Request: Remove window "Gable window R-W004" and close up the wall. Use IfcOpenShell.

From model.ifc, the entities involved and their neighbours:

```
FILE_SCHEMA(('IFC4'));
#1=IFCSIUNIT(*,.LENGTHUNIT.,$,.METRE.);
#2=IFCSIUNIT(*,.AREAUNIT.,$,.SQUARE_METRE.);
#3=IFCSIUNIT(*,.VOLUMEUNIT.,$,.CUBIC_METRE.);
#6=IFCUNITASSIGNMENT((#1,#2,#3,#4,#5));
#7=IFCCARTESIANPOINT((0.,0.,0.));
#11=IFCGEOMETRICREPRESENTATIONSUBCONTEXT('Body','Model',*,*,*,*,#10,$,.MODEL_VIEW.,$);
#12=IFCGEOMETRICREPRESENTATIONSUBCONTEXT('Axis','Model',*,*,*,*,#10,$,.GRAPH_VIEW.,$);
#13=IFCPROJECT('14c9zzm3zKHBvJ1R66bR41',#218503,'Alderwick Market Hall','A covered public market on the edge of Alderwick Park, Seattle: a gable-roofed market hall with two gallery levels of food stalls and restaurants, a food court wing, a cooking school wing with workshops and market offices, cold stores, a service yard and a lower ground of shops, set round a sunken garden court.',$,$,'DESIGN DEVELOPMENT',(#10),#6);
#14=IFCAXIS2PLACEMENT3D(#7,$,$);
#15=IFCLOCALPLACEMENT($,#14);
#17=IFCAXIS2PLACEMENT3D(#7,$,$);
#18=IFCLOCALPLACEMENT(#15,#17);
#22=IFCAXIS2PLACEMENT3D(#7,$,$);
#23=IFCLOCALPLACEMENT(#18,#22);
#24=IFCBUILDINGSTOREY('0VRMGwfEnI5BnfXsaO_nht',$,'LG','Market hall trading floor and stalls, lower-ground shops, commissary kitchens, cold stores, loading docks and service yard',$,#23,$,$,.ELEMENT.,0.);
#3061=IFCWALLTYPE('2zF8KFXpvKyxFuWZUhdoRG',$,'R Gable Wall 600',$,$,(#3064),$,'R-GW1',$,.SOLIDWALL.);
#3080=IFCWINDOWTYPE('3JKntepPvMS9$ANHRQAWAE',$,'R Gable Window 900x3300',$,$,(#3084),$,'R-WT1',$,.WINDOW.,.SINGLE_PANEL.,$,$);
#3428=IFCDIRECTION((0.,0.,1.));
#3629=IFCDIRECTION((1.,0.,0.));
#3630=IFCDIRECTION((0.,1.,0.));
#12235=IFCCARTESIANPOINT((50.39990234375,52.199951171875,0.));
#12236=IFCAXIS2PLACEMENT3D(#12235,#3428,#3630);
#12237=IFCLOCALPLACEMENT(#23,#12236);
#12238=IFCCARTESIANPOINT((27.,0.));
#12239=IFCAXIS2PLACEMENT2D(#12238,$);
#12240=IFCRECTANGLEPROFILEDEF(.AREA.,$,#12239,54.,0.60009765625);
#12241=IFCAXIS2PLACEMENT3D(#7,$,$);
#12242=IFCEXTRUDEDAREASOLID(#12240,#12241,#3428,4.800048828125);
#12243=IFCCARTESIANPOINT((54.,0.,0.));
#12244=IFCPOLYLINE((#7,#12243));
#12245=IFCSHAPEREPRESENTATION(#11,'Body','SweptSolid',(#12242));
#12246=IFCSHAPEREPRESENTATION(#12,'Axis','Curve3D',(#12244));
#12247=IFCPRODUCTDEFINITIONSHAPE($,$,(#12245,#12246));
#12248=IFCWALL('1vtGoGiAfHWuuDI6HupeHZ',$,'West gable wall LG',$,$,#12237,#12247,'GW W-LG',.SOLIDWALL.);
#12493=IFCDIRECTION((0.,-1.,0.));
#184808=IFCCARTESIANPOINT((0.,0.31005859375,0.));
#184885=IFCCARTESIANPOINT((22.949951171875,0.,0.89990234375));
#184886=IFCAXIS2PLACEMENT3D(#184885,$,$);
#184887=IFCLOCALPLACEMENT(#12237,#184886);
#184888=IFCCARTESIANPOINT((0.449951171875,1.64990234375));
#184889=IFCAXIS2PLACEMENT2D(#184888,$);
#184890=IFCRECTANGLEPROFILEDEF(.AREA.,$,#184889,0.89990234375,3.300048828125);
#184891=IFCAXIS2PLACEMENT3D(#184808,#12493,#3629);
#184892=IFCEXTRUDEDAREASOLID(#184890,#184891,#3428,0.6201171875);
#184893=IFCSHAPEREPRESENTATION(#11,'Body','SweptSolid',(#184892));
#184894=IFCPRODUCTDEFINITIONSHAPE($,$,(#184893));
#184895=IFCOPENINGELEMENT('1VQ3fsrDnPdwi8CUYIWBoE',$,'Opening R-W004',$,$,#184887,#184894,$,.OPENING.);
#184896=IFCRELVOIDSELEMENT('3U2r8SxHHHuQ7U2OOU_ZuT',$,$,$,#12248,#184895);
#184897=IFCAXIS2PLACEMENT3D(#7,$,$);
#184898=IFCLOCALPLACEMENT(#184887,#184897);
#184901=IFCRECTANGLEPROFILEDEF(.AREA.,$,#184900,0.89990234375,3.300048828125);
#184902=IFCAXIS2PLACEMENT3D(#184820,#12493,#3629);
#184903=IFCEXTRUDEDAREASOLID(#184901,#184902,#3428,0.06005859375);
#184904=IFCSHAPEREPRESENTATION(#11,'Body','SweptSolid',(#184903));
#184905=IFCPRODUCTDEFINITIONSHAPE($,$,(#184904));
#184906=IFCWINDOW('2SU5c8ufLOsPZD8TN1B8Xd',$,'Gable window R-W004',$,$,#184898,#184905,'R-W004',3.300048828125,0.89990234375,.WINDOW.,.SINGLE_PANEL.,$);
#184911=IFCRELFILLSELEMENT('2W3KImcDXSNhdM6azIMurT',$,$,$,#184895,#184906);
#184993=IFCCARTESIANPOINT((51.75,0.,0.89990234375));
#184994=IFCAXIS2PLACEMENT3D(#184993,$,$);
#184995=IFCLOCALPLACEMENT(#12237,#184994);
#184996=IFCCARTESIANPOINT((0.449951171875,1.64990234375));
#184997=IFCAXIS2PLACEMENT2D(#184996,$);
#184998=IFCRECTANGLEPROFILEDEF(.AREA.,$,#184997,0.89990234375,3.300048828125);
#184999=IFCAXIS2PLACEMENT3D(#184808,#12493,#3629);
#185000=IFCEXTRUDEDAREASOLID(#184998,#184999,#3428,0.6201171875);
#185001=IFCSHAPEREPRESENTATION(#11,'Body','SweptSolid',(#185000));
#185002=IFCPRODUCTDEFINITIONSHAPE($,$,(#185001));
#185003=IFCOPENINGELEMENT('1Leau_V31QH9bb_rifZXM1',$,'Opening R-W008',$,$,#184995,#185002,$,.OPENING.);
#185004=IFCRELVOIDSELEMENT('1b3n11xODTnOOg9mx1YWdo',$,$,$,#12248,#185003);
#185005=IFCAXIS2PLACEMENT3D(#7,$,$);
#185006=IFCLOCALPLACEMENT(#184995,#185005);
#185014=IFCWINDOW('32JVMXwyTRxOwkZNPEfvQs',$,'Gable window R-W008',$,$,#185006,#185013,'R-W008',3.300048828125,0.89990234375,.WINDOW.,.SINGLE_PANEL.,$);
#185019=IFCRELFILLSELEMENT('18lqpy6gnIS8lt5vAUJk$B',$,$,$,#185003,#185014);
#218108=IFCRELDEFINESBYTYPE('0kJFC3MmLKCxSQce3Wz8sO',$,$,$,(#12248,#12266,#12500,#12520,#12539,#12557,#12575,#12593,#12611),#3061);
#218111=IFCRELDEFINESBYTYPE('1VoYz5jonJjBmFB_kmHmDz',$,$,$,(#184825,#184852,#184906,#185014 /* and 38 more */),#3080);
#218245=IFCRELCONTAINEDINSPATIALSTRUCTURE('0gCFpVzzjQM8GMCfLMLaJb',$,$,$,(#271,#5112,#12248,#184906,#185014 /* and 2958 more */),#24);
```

```python
import ifcopenshell
import ifcopenshell.api.feature
import ifcopenshell.api.root
import ifcopenshell.geom
import ifcopenshell.util.shape

model = ifcopenshell.open("model.ifc")
settings = ifcopenshell.geom.settings()


def volume(element):
    """Net volume in cubic metres, openings subtracted."""
    shape = ifcopenshell.geom.create_shape(settings, element)
    return ifcopenshell.util.shape.get_volume(shape.geometry)


window = model.by_id(184906)
opening = window.FillsVoids[0].RelatingOpeningElement
wall = opening.VoidsElements[0].RelatingBuildingElement
before = volume(wall)

ifcopenshell.api.root.remove_product(model, product=window)
ifcopenshell.api.feature.remove_feature(model, feature=opening)

after = volume(wall)

print(f"wall volume {before:.3f} -> {after:.3f} m3")

model.write("model-out.ifc")
```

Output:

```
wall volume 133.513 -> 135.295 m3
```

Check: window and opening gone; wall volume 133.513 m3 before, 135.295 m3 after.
